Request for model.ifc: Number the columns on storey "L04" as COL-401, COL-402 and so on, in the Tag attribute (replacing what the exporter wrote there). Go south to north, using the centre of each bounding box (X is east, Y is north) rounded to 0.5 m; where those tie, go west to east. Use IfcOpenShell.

First a look at what the model holds.

```python
import ifcopenshell
import ifcopenshell.util.element
import ifcopenshell.util.placement

model = ifcopenshell.open("model.ifc")
print(model.schema)
storey = next(s for s in model.by_type("IfcBuildingStorey") if s.Name == "L04")
columns = [e for e in ifcopenshell.util.element.get_decomposition(storey) if e.is_a("IfcColumn")]
for e in sorted(columns, key=lambda e: e.id()):
    origin = ifcopenshell.util.placement.get_local_placement(e.ObjectPlacement)[:3, 3]
    print(e.id(), e.Tag, e.Name, origin.round(2) + 0.0, sep=" | ")
```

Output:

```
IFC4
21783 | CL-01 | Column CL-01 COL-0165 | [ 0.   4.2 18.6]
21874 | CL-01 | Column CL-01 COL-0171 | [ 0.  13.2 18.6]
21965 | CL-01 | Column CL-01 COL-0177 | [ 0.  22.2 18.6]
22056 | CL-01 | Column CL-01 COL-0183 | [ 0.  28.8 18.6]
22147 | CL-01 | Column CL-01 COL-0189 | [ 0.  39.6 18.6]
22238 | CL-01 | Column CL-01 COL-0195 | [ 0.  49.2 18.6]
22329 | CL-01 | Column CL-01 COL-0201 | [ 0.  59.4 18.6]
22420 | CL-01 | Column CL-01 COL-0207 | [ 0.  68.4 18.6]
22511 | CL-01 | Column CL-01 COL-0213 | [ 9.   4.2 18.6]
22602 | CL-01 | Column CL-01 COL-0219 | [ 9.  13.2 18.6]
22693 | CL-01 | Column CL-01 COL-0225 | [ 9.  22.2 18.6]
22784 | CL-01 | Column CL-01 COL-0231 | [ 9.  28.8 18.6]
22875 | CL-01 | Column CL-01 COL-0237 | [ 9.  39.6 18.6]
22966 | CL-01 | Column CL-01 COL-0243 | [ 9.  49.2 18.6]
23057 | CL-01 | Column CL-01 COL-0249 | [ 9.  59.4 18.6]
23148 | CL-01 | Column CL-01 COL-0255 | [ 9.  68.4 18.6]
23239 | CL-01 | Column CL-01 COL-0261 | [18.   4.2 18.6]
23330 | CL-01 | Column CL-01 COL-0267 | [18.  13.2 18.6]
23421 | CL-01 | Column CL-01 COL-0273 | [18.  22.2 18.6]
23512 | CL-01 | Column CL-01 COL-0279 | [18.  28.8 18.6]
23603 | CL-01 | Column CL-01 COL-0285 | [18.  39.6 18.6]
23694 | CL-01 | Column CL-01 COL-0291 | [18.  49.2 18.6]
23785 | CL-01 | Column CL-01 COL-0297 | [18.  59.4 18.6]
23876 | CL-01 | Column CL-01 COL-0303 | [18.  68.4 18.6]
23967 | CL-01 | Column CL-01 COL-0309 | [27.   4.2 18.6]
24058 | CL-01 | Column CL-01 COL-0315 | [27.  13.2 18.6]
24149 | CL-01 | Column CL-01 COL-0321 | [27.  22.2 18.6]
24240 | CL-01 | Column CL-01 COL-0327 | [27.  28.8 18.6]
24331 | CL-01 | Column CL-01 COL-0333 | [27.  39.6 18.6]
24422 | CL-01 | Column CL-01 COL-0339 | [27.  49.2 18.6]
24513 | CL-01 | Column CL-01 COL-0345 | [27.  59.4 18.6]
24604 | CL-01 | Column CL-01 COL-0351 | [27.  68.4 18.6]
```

```python
import ifcopenshell
import ifcopenshell.geom
import ifcopenshell.util.element
import ifcopenshell.util.shape

model = ifcopenshell.open("model.ifc")
settings = ifcopenshell.geom.settings()
settings.set("use-world-coords", True)


def centre(element):
    shape = ifcopenshell.geom.create_shape(settings, element)
    return ifcopenshell.util.shape.get_bbox_centroid(shape.geometry)


storey = next(s for s in model.by_type("IfcBuildingStorey") if s.Name == "L04")
columns = [e for e in ifcopenshell.util.element.get_decomposition(storey) if e.is_a("IfcColumn")]

# Insertion points can sit at a corner or the storey origin, so sort by the geometry (in metres).
centres = {e: centre(e) for e in columns}
columns.sort(key=lambda e: (round(centres[e][1] / 0.5), centres[e][0]))

for i, e in enumerate(columns, start=1):
    number = f"COL-4{i:02d}"
    e.Tag = number
    print(e.id(), number)

model.write("model_v2.ifc")
```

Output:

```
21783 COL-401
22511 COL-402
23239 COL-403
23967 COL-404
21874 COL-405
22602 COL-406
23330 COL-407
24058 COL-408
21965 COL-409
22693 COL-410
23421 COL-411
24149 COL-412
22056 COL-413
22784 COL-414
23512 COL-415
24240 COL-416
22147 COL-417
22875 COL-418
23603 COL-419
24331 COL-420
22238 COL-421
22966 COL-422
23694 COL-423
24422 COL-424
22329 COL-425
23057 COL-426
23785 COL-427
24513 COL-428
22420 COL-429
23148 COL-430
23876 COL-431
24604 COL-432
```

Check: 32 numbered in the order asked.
